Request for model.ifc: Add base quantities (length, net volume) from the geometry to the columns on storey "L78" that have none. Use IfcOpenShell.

First a look at what the model holds.

```python
import ifcopenshell
import ifcopenshell.util.element
import ifcopenshell.util.unit

model = ifcopenshell.open("model.ifc")
print(model.schema)
for unit_type in ("LENGTHUNIT", "AREAUNIT", "VOLUMEUNIT"):
    print(unit_type, ifcopenshell.util.unit.calculate_unit_scale(model, unit_type))
storey = next(s for s in model.by_type("IfcBuildingStorey") if s.Name == "L78")
columns = [e for e in ifcopenshell.util.element.get_decomposition(storey) if e.is_a("IfcColumn")]
for e in sorted(columns, key=lambda e: e.id()):
    print(e.id(), e.is_a(), e.Name, list(ifcopenshell.util.element.get_psets(e, qtos_only=True)), sep=" | ")
```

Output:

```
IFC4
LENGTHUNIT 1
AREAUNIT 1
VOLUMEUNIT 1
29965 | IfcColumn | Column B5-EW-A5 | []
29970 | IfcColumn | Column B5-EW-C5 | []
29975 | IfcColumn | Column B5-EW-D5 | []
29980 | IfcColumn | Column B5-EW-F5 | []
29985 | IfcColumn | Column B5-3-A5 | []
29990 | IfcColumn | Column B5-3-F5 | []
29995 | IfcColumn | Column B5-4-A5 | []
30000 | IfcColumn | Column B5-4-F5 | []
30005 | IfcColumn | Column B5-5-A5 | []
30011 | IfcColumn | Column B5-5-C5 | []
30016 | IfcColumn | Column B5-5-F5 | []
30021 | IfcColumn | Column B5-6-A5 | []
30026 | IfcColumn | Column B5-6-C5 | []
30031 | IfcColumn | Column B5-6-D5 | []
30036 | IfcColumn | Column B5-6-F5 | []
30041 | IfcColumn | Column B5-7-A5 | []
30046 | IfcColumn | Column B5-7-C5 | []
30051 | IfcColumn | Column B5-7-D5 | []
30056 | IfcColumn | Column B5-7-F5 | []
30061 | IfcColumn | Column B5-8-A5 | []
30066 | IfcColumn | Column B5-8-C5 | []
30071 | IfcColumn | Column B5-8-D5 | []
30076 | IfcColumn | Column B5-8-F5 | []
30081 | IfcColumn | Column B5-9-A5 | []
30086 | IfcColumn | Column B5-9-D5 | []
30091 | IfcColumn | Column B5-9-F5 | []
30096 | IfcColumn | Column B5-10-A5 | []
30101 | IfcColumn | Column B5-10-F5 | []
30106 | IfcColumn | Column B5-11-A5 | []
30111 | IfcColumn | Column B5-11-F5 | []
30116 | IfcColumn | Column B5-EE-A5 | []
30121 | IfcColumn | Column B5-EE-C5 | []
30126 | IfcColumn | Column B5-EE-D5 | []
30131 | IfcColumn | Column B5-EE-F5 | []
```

```python
import ifcopenshell
import ifcopenshell.api.pset
import ifcopenshell.geom
import ifcopenshell.util.element
import ifcopenshell.util.shape
import ifcopenshell.util.unit

model = ifcopenshell.open("model.ifc")
unit_scale = ifcopenshell.util.unit.calculate_unit_scale(model)
volume_scale = ifcopenshell.util.unit.calculate_unit_scale(model, "VOLUMEUNIT")
settings = ifcopenshell.geom.settings()

storey = next(s for s in model.by_type("IfcBuildingStorey") if s.Name == "L78")
columns = [e for e in ifcopenshell.util.element.get_decomposition(storey) if e.is_a("IfcColumn")]

for e in sorted(columns, key=lambda e: e.id()):
    if ifcopenshell.util.element.get_psets(e, qtos_only=True, should_inherit=False):
        continue
    # Geometry comes back in metres, in the element's own axes.
    shape = ifcopenshell.geom.create_shape(settings, e)
    values = {
        "Length": ifcopenshell.util.shape.get_z(shape.geometry) / unit_scale,
        "NetVolume": ifcopenshell.util.shape.get_volume(shape.geometry) / volume_scale,
    }
    qto = ifcopenshell.api.pset.add_qto(model, product=e, name="Qto_ColumnBaseQuantities")
    ifcopenshell.api.pset.edit_qto(model, qto=qto, properties=values)
    print(e.id(), {k: round(v, 3) for k, v in values.items()})

model.write("model-out.ifc")
```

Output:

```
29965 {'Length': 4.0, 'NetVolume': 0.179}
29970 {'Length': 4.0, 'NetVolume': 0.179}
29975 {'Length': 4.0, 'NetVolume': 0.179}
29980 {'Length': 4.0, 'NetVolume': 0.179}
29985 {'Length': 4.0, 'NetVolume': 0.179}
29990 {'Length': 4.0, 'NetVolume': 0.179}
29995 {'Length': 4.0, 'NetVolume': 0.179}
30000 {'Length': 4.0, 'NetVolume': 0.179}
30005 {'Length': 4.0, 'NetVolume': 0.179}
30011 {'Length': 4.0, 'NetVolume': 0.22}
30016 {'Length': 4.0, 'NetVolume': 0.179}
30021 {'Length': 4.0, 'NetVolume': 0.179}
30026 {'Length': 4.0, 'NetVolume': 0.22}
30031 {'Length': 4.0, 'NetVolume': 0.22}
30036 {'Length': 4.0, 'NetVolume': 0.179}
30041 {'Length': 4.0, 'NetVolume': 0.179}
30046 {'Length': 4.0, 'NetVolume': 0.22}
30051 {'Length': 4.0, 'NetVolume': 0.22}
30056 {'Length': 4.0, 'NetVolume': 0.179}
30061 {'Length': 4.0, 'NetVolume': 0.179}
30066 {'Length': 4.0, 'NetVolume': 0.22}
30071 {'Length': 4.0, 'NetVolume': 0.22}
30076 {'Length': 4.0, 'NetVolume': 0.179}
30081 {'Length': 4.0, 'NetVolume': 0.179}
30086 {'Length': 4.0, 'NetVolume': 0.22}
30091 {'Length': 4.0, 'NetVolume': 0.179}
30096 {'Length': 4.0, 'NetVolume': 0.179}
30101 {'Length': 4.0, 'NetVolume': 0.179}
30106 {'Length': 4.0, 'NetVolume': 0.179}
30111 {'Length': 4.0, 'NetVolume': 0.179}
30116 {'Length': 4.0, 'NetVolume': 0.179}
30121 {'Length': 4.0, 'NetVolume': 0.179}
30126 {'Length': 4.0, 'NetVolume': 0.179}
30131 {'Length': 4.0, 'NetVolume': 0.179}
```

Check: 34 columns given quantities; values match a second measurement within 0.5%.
